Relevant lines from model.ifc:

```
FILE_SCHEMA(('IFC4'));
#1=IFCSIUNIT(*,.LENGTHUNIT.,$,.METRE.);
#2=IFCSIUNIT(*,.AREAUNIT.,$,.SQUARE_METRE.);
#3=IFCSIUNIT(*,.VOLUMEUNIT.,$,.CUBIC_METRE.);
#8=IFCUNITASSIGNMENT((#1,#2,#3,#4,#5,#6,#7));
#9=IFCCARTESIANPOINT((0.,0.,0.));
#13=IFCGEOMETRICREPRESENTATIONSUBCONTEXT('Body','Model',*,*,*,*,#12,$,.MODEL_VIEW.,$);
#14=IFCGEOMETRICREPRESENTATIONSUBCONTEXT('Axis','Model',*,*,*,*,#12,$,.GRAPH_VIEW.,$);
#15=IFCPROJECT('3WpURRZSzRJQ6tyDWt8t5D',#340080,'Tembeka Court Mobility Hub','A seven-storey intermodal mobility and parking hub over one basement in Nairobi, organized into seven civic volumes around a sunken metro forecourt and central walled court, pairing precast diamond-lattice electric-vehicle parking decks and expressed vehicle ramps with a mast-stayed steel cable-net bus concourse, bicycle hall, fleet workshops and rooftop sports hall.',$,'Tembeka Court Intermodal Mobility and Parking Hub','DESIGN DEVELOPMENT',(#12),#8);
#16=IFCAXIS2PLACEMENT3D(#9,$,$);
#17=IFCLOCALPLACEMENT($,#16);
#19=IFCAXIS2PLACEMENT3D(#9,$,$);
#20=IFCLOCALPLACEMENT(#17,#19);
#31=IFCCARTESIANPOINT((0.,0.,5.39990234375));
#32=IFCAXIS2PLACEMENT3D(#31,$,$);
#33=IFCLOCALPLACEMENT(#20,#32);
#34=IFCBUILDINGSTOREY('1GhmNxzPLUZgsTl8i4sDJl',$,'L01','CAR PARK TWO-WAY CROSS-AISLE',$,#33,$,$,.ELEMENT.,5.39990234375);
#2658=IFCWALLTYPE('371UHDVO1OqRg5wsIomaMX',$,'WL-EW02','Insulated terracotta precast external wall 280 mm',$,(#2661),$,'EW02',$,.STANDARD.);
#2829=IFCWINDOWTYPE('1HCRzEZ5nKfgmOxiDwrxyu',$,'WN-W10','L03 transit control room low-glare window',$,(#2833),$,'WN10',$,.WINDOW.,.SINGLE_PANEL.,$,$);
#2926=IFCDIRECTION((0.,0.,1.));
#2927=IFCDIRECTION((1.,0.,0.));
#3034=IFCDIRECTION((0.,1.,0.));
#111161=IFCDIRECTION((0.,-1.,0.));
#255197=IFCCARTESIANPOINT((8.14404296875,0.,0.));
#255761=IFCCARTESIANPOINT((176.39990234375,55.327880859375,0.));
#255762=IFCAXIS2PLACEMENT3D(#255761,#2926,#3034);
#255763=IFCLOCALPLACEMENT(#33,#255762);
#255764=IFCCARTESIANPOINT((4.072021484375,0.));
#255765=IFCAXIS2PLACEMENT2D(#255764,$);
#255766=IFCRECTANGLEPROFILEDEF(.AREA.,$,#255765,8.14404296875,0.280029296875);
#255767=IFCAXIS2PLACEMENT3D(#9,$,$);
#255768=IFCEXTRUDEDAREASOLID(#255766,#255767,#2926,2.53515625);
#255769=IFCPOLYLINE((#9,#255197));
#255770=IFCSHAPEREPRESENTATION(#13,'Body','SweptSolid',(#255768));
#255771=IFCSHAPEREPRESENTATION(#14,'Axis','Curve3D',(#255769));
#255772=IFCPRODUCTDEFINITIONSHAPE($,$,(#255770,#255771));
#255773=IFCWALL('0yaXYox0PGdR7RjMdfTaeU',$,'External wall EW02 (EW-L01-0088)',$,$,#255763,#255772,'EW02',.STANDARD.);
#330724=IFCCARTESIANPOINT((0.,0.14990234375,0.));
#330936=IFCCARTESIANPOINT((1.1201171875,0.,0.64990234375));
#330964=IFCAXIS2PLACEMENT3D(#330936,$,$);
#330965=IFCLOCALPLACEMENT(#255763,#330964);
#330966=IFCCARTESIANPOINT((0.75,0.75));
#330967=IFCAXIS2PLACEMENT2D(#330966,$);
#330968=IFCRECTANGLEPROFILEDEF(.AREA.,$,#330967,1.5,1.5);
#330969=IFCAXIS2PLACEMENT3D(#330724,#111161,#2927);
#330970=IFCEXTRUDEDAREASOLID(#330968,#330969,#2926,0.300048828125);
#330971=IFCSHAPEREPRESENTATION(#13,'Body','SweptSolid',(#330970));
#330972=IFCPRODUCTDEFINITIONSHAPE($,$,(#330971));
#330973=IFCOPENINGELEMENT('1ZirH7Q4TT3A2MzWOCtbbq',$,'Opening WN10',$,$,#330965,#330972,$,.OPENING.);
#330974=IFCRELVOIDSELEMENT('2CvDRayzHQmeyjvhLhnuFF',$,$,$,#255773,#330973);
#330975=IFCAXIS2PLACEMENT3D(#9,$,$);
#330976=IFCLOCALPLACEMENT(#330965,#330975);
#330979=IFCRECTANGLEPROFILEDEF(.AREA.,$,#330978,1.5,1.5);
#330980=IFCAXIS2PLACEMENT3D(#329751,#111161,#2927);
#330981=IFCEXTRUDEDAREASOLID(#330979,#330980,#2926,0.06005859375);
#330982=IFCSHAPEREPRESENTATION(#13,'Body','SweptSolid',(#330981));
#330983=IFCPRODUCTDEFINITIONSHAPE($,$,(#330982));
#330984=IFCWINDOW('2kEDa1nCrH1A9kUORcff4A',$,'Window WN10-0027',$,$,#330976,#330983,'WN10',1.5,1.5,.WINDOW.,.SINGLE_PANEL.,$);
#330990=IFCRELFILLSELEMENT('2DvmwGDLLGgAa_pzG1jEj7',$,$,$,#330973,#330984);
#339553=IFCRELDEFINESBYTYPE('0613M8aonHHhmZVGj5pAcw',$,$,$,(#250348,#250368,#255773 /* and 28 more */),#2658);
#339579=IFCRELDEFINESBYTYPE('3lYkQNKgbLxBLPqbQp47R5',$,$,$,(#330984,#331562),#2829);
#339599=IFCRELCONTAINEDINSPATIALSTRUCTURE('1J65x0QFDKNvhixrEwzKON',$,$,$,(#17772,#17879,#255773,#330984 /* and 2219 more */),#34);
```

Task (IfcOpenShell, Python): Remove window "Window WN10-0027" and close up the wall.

```python
import ifcopenshell
import ifcopenshell.api.feature
import ifcopenshell.api.root
import ifcopenshell.geom
import ifcopenshell.util.shape

model = ifcopenshell.open("model.ifc")
settings = ifcopenshell.geom.settings()


def volume(element):
    """Net volume in cubic metres, openings subtracted."""
    shape = ifcopenshell.geom.create_shape(settings, element)
    return ifcopenshell.util.shape.get_volume(shape.geometry)


window = model.by_guid("2kEDa1nCrH1A9kUORcff4A")
opening = window.FillsVoids[0].RelatingOpeningElement
wall = opening.VoidsElements[0].RelatingBuildingElement
before = volume(wall)

ifcopenshell.api.root.remove_product(model, product=window)
ifcopenshell.api.feature.remove_feature(model, feature=opening)

after = volume(wall)

print(f"wall volume {before:.3f} -> {after:.3f} m3")

model.write("model-out.ifc")
```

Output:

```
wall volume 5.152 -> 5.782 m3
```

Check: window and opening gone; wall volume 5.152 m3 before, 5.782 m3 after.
